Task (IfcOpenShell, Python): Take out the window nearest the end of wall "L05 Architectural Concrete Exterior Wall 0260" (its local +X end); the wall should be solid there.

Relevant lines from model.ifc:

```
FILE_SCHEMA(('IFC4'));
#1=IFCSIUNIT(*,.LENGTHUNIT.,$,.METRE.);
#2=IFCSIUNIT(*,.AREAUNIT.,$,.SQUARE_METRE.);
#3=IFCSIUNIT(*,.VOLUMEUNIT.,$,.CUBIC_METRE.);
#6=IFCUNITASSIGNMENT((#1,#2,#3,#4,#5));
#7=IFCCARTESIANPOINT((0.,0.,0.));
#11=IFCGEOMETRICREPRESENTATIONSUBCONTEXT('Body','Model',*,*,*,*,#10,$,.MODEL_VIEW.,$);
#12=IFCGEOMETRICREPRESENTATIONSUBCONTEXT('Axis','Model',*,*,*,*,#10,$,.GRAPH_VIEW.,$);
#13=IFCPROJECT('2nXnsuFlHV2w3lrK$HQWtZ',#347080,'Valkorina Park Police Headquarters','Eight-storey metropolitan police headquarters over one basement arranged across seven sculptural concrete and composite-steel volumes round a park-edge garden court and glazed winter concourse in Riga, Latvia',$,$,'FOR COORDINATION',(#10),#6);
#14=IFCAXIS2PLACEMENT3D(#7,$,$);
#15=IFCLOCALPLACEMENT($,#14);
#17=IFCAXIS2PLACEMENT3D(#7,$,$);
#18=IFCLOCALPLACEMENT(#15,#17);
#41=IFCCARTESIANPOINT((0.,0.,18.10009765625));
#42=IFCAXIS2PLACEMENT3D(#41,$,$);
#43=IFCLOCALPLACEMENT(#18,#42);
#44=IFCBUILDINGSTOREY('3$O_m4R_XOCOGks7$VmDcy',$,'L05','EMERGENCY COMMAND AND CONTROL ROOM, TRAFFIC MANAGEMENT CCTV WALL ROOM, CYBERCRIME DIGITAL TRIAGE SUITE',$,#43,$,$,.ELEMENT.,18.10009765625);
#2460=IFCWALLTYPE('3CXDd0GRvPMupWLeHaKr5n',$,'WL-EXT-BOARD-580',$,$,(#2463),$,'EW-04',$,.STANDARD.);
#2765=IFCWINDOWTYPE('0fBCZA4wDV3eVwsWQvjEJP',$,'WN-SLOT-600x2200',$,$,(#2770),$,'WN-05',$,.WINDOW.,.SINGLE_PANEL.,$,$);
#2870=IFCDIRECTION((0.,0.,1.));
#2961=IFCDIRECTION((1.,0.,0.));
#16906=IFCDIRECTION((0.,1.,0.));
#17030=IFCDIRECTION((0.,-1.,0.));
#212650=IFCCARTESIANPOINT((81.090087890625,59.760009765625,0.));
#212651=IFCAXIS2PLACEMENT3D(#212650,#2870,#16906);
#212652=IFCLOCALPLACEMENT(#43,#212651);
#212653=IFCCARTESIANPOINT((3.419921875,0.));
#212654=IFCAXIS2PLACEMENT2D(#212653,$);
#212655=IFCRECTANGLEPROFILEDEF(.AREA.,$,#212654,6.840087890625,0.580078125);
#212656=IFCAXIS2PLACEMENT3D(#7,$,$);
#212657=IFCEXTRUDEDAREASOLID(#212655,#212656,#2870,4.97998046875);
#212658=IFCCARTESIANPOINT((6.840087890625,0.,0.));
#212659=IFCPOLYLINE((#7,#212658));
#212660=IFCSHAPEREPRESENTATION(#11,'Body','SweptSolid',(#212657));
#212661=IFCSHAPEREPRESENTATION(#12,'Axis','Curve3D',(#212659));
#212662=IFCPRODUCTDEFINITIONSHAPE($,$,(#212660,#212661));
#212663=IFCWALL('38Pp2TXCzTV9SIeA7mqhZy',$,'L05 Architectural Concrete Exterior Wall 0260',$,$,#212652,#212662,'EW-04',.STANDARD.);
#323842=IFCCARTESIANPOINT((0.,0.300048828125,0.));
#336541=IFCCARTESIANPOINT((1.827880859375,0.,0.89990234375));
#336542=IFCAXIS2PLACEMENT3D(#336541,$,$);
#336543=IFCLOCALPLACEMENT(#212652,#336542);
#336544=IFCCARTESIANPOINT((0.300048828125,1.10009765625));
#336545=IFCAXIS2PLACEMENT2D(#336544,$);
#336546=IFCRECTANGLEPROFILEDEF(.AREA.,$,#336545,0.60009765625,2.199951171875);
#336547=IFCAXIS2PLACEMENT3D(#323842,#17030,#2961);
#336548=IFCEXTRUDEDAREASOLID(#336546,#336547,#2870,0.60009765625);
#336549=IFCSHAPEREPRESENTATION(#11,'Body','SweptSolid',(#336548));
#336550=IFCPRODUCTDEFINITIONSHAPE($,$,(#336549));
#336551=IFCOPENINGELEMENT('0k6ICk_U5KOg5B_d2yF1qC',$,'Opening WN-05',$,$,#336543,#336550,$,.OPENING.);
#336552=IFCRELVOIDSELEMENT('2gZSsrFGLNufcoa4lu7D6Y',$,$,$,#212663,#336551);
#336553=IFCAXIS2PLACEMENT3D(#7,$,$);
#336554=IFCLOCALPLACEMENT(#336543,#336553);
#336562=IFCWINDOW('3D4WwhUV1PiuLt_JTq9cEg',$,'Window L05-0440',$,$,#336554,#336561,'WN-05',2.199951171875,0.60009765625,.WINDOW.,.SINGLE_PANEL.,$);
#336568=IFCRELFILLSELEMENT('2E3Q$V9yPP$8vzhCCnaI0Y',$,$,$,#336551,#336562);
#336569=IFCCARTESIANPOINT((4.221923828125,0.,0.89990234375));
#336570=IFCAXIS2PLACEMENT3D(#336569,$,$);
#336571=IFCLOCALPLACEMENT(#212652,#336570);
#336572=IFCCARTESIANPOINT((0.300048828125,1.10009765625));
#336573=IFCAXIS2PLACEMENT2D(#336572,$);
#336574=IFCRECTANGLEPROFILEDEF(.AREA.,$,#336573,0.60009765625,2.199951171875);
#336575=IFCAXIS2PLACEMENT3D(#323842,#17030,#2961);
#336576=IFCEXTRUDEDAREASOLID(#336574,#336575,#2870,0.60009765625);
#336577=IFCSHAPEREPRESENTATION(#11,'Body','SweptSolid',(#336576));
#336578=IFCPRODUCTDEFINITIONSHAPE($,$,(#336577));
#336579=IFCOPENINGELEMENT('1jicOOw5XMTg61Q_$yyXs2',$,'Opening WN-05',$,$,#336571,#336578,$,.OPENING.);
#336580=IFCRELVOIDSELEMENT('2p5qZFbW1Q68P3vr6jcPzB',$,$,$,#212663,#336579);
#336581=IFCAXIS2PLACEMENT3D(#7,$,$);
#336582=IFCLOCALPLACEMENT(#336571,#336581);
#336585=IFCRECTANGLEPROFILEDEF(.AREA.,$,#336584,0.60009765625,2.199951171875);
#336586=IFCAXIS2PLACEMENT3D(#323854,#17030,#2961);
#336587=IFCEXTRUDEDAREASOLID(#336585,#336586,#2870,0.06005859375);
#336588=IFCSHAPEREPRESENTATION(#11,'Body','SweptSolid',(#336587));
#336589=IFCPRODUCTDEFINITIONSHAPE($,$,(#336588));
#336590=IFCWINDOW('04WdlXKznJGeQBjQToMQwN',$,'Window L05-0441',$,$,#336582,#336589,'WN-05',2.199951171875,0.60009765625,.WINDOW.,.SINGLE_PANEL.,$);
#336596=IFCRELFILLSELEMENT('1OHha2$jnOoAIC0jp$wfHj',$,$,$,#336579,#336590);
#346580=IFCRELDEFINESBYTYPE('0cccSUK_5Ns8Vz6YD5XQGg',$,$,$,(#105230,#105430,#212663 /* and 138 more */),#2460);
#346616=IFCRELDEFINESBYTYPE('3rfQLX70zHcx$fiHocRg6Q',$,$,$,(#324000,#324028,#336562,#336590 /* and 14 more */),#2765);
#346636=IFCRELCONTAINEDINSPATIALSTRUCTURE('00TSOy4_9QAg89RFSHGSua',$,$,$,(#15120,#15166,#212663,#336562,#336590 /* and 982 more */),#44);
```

```python
import ifcopenshell
import ifcopenshell.api.feature
import ifcopenshell.api.root
import ifcopenshell.geom
import ifcopenshell.util.shape

model = ifcopenshell.open("model.ifc")
settings = ifcopenshell.geom.settings()


def volume(element):
    """Net volume in cubic metres, openings subtracted."""
    shape = ifcopenshell.geom.create_shape(settings, element)
    return ifcopenshell.util.shape.get_volume(shape.geometry)


window = model.by_id(336590)
opening = window.FillsVoids[0].RelatingOpeningElement
wall = opening.VoidsElements[0].RelatingBuildingElement
before = volume(wall)

ifcopenshell.api.root.remove_product(model, product=window)
ifcopenshell.api.feature.remove_feature(model, feature=opening)

after = volume(wall)

print(f"wall volume {before:.3f} -> {after:.3f} m3")

model.write("model_v2.ifc")
```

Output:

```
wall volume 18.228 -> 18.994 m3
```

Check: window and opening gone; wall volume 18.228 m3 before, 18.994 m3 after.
